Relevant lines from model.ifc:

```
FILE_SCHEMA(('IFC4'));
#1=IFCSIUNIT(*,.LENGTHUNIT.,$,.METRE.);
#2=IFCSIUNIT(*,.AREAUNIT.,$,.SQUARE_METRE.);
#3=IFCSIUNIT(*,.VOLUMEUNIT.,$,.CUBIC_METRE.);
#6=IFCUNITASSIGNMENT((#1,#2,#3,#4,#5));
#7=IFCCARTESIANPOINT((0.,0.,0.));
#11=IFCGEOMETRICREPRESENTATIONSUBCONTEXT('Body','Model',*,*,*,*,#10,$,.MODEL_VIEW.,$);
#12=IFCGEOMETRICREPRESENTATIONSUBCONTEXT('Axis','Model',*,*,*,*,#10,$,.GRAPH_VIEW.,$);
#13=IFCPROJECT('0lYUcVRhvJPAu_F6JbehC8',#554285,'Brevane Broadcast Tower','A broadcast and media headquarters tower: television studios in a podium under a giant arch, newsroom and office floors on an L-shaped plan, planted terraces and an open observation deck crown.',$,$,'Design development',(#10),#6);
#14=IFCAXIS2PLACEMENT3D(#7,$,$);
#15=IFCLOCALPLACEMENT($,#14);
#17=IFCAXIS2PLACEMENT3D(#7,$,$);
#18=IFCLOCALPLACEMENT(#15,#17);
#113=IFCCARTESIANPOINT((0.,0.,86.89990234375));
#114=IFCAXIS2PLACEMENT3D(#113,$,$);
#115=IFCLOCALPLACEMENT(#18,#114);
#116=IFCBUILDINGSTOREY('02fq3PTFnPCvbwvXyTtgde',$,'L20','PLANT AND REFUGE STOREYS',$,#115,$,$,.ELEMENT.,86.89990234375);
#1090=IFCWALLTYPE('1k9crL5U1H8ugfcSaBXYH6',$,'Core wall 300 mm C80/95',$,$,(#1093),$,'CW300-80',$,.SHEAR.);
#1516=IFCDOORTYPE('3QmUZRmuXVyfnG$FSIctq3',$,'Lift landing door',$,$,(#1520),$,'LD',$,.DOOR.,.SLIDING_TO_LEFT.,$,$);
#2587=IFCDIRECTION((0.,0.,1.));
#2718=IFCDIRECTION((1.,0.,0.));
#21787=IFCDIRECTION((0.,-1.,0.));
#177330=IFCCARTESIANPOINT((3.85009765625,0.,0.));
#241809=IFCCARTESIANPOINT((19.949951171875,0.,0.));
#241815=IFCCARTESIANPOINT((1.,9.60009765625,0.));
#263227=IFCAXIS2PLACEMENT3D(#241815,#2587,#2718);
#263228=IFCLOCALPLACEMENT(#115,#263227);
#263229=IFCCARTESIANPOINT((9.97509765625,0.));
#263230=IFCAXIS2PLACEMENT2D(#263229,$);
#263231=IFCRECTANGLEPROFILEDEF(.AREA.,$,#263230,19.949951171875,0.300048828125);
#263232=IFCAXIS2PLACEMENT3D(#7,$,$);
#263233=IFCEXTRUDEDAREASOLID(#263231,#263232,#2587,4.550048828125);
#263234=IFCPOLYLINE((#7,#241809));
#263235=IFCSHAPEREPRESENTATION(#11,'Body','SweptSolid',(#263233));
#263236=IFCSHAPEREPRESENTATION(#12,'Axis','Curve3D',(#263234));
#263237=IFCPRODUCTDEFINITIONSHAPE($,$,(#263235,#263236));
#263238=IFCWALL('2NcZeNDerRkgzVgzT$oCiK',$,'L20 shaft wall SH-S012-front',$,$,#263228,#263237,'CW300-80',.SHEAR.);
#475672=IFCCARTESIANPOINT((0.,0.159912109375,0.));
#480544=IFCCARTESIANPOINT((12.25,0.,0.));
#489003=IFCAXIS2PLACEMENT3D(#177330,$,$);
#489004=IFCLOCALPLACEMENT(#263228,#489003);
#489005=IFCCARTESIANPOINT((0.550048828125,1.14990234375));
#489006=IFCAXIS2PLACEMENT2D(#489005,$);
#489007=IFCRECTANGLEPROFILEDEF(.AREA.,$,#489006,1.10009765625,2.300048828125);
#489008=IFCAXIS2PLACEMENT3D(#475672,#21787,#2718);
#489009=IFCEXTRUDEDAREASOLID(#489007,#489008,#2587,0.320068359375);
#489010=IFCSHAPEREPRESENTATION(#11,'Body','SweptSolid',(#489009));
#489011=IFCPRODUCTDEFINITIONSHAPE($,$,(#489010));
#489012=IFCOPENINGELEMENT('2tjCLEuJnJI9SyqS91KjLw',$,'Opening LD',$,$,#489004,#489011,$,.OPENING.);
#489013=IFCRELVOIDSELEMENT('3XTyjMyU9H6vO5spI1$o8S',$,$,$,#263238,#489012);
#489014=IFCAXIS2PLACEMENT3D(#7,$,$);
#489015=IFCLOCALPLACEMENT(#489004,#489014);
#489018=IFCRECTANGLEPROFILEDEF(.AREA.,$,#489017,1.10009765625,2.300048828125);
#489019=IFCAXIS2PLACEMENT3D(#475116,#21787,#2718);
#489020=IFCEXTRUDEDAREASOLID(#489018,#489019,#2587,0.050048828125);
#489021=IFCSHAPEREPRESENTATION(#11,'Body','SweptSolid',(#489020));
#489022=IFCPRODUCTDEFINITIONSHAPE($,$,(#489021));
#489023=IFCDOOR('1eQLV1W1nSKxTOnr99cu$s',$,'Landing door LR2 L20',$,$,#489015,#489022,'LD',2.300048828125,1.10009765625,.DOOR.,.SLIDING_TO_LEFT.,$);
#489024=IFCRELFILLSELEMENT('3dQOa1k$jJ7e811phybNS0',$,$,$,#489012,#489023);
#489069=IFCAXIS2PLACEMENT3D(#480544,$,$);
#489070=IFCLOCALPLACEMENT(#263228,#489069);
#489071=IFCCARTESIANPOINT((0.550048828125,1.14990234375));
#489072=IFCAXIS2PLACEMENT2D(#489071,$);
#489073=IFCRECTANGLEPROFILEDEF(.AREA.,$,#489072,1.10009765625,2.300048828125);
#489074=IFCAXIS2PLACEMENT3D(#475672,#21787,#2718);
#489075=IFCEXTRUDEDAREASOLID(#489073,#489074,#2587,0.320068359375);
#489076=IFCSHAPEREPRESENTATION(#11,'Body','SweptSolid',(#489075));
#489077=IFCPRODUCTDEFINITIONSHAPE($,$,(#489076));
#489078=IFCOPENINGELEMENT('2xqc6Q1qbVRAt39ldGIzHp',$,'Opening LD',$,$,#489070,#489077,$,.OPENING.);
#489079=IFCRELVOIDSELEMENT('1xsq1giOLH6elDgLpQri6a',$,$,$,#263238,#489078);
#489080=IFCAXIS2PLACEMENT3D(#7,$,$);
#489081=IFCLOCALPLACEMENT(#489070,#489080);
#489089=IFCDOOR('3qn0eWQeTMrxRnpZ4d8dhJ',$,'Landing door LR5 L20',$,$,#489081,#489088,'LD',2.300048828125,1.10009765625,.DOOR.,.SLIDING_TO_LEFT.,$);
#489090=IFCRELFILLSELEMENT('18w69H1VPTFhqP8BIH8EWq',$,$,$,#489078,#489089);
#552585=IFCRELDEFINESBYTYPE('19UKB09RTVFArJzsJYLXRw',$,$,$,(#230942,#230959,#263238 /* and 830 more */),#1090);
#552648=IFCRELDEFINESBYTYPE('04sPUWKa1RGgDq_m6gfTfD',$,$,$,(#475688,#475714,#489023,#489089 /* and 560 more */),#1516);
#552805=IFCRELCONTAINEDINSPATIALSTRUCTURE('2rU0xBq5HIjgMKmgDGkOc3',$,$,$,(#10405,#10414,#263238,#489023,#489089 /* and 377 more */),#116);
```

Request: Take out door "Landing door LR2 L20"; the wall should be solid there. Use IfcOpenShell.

```python
import ifcopenshell
import ifcopenshell.api.feature
import ifcopenshell.api.root
import ifcopenshell.geom
import ifcopenshell.util.shape

model = ifcopenshell.open("model.ifc")
settings = ifcopenshell.geom.settings()


def volume(element):
    """Net volume in cubic metres, openings subtracted."""
    shape = ifcopenshell.geom.create_shape(settings, element)
    return ifcopenshell.util.shape.get_volume(shape.geometry)


door = model.by_id(489023)
opening = door.FillsVoids[0].RelatingOpeningElement
wall = opening.VoidsElements[0].RelatingBuildingElement
before = volume(wall)

ifcopenshell.api.root.remove_product(model, product=door)
ifcopenshell.api.feature.remove_feature(model, feature=opening)

after = volume(wall)

print(f"wall volume {before:.3f} -> {after:.3f} m3")

model.write("model_edited.ifc")
```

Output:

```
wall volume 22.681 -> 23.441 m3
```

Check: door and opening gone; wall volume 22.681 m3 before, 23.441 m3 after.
